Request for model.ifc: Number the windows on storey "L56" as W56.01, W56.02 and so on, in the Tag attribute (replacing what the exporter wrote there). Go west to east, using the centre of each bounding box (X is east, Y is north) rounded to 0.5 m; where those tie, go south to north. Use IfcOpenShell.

First a look at what the model holds.

```python
import ifcopenshell
import ifcopenshell.util.element
import ifcopenshell.util.placement

model = ifcopenshell.open("model.ifc")
print(model.schema)
storey = next(s for s in model.by_type("IfcBuildingStorey") if s.Name == "L56")
windows = [e for e in ifcopenshell.util.element.get_decomposition(storey) if e.is_a("IfcWindow")]
for e in sorted(windows, key=lambda e: e.id()):
    origin = ifcopenshell.util.placement.get_local_placement(e.ObjectPlacement)[:3, 3]
    print(e.id(), e.Tag, e.Name, origin.round(2) + 0.0, sep=" | ")
```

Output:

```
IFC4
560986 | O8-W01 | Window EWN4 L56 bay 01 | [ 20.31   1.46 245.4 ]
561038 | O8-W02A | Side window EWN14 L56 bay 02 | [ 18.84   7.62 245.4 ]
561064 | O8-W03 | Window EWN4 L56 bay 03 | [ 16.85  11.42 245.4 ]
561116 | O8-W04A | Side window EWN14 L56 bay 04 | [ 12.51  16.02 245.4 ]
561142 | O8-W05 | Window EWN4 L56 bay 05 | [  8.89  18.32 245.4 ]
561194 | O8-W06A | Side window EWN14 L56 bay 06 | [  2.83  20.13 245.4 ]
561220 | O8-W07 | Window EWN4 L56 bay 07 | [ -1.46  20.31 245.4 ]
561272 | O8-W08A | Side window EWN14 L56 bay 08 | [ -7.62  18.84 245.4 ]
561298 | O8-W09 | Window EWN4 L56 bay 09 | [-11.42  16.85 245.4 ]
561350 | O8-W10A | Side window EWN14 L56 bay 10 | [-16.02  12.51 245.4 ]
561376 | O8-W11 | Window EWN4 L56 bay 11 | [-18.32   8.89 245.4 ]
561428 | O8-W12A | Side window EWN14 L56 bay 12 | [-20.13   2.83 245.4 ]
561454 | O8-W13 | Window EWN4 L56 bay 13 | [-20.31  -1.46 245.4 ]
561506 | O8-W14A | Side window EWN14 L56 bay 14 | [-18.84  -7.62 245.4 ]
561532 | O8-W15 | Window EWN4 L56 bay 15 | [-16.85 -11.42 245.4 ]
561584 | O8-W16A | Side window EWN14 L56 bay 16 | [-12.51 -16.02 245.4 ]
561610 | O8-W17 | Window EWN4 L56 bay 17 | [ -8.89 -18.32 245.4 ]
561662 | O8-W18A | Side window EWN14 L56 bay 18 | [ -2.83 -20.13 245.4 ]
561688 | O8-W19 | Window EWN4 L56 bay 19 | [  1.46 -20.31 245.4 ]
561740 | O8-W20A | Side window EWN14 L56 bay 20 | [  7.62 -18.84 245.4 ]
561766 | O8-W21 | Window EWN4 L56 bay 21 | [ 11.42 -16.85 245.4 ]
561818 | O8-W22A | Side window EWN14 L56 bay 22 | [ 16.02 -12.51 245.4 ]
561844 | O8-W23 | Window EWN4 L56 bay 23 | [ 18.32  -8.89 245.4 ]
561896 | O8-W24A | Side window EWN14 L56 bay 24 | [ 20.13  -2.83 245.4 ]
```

```python
import ifcopenshell
import ifcopenshell.geom
import ifcopenshell.util.element
import ifcopenshell.util.shape

model = ifcopenshell.open("model.ifc")
settings = ifcopenshell.geom.settings()
settings.set("use-world-coords", True)


def centre(element):
    shape = ifcopenshell.geom.create_shape(settings, element)
    return ifcopenshell.util.shape.get_bbox_centroid(shape.geometry)


storey = next(s for s in model.by_type("IfcBuildingStorey") if s.Name == "L56")
windows = [e for e in ifcopenshell.util.element.get_decomposition(storey) if e.is_a("IfcWindow")]

# Insertion points can sit at a corner or the storey origin, so sort by the geometry (in metres).
centres = {e: centre(e) for e in windows}
windows.sort(key=lambda e: (round(centres[e][0] / 0.5), centres[e][1]))

for i, e in enumerate(windows, start=1):
    number = f"W56.{i:02d}"
    e.Tag = number
    print(e.id(), number)

model.write("model_rev.ifc")
```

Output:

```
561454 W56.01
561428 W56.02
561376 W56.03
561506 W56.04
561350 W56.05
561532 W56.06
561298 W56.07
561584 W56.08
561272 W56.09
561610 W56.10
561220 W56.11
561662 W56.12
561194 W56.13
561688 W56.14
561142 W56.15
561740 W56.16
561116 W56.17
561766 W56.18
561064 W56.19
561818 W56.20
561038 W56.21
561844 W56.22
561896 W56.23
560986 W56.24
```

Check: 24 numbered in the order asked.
